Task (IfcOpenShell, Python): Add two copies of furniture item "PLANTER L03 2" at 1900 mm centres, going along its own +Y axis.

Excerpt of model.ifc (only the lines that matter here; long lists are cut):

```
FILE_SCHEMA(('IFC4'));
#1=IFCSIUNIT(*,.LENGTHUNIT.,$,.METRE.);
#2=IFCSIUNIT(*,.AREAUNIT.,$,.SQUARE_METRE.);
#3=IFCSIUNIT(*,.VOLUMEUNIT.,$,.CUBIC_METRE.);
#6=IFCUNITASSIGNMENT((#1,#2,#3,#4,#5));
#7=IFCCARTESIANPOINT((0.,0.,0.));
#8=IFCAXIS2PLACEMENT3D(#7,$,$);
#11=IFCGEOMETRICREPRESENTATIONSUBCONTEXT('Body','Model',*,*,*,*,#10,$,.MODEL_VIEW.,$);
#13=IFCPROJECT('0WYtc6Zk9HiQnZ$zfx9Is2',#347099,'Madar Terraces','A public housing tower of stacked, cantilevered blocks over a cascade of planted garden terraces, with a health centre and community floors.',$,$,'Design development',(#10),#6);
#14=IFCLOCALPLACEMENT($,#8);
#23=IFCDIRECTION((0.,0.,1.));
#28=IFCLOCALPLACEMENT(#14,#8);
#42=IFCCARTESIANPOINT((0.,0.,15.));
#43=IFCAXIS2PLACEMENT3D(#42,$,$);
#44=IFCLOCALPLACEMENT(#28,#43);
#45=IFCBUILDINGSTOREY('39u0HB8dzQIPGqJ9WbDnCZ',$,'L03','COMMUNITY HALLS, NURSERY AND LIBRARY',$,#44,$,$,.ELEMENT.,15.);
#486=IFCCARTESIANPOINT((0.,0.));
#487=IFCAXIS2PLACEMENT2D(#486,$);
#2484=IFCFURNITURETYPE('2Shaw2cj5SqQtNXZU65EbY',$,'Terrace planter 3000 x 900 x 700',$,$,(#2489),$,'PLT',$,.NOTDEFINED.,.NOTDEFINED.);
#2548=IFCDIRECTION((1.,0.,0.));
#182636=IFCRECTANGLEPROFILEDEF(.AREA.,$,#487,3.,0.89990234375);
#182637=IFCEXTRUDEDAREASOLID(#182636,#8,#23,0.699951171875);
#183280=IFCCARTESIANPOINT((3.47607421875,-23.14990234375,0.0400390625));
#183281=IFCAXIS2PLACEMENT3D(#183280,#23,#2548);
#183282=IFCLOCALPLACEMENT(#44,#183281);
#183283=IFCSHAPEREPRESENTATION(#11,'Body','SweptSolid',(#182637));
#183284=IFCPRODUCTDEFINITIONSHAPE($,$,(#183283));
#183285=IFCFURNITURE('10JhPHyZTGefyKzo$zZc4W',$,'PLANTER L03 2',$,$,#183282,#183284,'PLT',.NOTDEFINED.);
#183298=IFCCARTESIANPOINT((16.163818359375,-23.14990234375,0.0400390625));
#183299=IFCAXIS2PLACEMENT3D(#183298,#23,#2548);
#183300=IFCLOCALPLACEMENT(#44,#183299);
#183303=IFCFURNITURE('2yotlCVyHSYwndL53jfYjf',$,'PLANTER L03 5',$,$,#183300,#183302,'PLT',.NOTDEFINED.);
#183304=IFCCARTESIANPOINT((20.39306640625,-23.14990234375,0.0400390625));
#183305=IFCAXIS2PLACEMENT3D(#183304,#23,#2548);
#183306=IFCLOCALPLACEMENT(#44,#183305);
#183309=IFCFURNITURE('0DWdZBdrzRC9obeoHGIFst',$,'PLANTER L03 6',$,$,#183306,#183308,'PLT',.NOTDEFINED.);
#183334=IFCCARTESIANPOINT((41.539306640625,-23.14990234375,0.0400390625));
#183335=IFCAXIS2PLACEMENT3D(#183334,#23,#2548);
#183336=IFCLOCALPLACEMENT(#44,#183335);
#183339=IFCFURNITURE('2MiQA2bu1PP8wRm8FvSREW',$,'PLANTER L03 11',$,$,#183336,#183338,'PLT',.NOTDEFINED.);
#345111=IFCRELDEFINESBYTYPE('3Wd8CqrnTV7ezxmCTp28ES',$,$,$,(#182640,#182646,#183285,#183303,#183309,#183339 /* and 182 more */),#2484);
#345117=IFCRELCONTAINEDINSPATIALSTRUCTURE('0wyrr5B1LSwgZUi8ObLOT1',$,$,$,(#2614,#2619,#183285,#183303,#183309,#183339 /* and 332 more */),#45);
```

```python
import ifcopenshell
import ifcopenshell.api.geometry
import ifcopenshell.api.root
import ifcopenshell.util.element
import ifcopenshell.util.placement
import ifcopenshell.util.unit

model = ifcopenshell.open("model.ifc")
unit_scale = ifcopenshell.util.unit.calculate_unit_scale(model)

source = model.by_guid("10JhPHyZTGefyKzo$zZc4W")
base = ifcopenshell.util.placement.get_local_placement(source.ObjectPlacement)
step = base[:3, 1] * 1.9 / unit_scale

for i in range(1, 3):
    copy = ifcopenshell.api.root.copy_class(model, product=source)
    copy.Representation = ifcopenshell.util.element.copy_deep(
        model, source.Representation, exclude=["IfcGeometricRepresentationContext", "IfcRepresentationMap"]
    )
    copy.Tag = None
    matrix = base.copy()
    matrix[:3, 3] += i * step
    print("added at", matrix[:3, 3].round(3) + 0.0)
    ifcopenshell.api.geometry.edit_object_placement(model, product=copy, matrix=matrix, is_si=False)

model.write("model_updated.ifc")
```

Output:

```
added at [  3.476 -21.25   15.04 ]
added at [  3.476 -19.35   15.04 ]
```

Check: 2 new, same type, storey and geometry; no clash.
